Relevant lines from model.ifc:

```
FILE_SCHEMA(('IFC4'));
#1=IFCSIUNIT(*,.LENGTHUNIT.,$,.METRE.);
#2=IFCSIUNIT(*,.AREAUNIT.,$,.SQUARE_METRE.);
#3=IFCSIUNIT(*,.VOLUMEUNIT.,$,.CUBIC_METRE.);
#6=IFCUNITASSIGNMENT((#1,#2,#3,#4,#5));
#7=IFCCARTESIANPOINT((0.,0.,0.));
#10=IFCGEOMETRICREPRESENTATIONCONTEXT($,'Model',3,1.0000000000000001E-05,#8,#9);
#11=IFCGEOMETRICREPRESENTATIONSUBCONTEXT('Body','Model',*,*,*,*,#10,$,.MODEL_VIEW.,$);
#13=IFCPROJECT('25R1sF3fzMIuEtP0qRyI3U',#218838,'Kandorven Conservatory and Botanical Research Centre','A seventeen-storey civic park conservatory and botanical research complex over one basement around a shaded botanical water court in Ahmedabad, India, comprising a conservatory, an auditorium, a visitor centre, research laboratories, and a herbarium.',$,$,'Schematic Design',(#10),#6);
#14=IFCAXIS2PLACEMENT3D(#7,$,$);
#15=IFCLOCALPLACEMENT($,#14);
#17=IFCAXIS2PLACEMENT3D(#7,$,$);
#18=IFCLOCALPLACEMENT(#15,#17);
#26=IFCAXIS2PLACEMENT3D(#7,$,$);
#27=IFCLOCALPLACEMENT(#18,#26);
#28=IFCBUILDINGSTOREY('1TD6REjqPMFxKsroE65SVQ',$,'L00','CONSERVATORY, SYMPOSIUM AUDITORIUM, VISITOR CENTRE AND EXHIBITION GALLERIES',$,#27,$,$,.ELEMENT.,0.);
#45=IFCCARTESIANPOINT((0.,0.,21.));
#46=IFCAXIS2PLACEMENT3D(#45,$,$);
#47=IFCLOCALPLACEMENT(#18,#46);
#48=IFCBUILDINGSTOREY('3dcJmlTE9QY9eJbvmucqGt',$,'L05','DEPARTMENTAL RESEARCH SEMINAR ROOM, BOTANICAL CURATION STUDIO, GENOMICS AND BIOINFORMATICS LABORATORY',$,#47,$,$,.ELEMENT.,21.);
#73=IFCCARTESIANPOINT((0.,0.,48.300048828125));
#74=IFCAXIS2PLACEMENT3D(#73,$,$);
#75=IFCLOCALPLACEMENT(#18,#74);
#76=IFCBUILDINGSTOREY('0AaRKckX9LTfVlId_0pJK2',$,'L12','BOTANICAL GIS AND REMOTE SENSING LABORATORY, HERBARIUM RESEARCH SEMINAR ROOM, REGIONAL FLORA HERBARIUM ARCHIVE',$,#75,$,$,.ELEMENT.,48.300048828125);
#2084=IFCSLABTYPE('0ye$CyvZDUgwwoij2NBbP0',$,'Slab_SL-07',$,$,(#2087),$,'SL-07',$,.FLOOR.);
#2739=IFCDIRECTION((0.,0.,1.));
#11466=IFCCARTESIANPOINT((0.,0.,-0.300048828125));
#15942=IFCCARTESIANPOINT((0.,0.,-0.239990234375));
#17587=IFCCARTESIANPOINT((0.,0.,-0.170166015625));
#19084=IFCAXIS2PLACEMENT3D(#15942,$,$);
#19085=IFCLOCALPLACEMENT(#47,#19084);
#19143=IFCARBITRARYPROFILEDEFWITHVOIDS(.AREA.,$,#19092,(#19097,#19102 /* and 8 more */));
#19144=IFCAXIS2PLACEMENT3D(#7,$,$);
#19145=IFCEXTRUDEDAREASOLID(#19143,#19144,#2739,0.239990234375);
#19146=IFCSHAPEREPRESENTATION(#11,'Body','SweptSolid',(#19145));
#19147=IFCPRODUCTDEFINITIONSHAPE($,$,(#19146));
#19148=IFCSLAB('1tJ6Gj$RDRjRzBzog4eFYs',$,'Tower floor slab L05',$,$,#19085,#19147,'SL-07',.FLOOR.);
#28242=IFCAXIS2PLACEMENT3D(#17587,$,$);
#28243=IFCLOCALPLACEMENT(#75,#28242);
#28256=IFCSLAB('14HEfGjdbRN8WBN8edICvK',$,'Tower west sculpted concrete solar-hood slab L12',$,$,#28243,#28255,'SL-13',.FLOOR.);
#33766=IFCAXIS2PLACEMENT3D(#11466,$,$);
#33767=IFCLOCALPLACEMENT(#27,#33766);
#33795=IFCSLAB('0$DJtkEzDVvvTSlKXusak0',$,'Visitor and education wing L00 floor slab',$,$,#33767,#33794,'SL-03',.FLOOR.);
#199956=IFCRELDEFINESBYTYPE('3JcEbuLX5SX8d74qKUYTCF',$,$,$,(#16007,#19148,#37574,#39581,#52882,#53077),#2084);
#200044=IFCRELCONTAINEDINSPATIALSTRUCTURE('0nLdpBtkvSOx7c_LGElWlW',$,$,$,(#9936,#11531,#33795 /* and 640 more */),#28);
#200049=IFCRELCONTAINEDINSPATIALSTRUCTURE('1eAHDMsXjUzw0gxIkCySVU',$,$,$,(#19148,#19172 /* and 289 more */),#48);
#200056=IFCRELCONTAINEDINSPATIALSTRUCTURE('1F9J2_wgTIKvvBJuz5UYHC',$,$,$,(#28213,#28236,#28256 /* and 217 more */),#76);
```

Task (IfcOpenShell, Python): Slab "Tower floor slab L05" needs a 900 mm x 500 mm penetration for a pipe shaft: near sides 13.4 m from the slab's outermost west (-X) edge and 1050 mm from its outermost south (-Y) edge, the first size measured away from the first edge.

```python
import numpy as np
import ifcopenshell
import ifcopenshell.api.feature
import ifcopenshell.api.geometry
import ifcopenshell.api.root
import ifcopenshell.geom
import ifcopenshell.util.placement
import ifcopenshell.util.representation
import ifcopenshell.util.shape
import ifcopenshell.util.unit

model = ifcopenshell.open("model.ifc")
unit_scale = ifcopenshell.util.unit.calculate_unit_scale(model)
settings = ifcopenshell.geom.settings()


def volume(element):
    """Net volume in cubic metres, openings subtracted."""
    shape = ifcopenshell.geom.create_shape(settings, element)
    return ifcopenshell.util.shape.get_volume(shape.geometry)


slab = model.by_guid("1tJ6Gj$RDRjRzBzog4eFYs")
before = volume(slab)

# Extent in the slab's own axes, in metres. The edges named are its -X and -Y sides.
slab_shape = ifcopenshell.geom.create_shape(settings, slab)
vertices = ifcopenshell.util.shape.get_vertices(slab_shape.geometry)
x_min, y_min, bottom = vertices.min(axis=0)
top = vertices[:, 2].max()

opening = ifcopenshell.api.root.create_entity(model, ifc_class="IfcOpeningElement", name="Pipe shaft opening", predefined_type="OPENING")
context = ifcopenshell.util.representation.get_context(model, "Model", "Body", "MODEL_VIEW")
width, depth = 0.9, 0.5
outline = [(0.0, 0.0), (width, 0.0), (width, depth), (0.0, depth), (0.0, 0.0)]
# Overshoot both faces by 50 mm so the cut is clean.
shape = ifcopenshell.api.geometry.add_slab_representation(
    model, context=context, depth=top - bottom + 0.1, polyline=outline
)
ifcopenshell.api.geometry.assign_representation(model, product=opening, representation=shape)

matrix = ifcopenshell.util.placement.get_local_placement(slab.ObjectPlacement)
matrix[:, 3] = matrix @ np.append(np.array([x_min + 13.4, y_min + 1.05, bottom - 0.05]) / unit_scale, 1.0)
ifcopenshell.api.geometry.edit_object_placement(model, product=opening, matrix=matrix, is_si=False)
ifcopenshell.api.feature.add_feature(model, feature=opening, element=slab)

after = volume(slab)

print(f"slab volume {before:.3f} -> {after:.3f} m3")

model.write("model_updated.ifc")
```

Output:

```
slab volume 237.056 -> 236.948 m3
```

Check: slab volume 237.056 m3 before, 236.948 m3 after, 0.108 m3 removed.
